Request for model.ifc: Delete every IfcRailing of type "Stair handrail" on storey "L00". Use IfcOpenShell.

First a look at what the model holds.

```python
import ifcopenshell
import ifcopenshell.util.element

model = ifcopenshell.open("model.ifc")
print(model.schema)
storey = next(s for s in model.by_type("IfcBuildingStorey") if s.Name == "L00")
railings = [e for e in ifcopenshell.util.element.get_decomposition(storey) if e.is_a("IfcRailing")]
seen = {}
for e in railings:
    element_type = ifcopenshell.util.element.get_type(e)
    name = element_type.Name if element_type not in (None, e) else None
    seen[name] = seen.get(name, 0) + 1
for name, count in sorted(seen.items(), key=str):
    print(count, "x", name)
```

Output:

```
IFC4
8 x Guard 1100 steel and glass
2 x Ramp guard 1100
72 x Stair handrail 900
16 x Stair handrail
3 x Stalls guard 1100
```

```python
import ifcopenshell
import ifcopenshell.api.root
import ifcopenshell.util.element

model = ifcopenshell.open("model.ifc")

storey = next(s for s in model.by_type("IfcBuildingStorey") if s.Name == "L00")
railings = [e for e in ifcopenshell.util.element.get_decomposition(storey) if e.is_a("IfcRailing")]
targets = [e for e in railings if (t := ifcopenshell.util.element.get_type(e)) not in (None, e) and t.Name == "Stair handrail"]

for e in targets:
    ifcopenshell.api.root.remove_product(model, product=e)
print(len(targets), "removed")

model.write("model-out.ifc")
```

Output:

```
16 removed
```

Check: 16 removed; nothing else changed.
